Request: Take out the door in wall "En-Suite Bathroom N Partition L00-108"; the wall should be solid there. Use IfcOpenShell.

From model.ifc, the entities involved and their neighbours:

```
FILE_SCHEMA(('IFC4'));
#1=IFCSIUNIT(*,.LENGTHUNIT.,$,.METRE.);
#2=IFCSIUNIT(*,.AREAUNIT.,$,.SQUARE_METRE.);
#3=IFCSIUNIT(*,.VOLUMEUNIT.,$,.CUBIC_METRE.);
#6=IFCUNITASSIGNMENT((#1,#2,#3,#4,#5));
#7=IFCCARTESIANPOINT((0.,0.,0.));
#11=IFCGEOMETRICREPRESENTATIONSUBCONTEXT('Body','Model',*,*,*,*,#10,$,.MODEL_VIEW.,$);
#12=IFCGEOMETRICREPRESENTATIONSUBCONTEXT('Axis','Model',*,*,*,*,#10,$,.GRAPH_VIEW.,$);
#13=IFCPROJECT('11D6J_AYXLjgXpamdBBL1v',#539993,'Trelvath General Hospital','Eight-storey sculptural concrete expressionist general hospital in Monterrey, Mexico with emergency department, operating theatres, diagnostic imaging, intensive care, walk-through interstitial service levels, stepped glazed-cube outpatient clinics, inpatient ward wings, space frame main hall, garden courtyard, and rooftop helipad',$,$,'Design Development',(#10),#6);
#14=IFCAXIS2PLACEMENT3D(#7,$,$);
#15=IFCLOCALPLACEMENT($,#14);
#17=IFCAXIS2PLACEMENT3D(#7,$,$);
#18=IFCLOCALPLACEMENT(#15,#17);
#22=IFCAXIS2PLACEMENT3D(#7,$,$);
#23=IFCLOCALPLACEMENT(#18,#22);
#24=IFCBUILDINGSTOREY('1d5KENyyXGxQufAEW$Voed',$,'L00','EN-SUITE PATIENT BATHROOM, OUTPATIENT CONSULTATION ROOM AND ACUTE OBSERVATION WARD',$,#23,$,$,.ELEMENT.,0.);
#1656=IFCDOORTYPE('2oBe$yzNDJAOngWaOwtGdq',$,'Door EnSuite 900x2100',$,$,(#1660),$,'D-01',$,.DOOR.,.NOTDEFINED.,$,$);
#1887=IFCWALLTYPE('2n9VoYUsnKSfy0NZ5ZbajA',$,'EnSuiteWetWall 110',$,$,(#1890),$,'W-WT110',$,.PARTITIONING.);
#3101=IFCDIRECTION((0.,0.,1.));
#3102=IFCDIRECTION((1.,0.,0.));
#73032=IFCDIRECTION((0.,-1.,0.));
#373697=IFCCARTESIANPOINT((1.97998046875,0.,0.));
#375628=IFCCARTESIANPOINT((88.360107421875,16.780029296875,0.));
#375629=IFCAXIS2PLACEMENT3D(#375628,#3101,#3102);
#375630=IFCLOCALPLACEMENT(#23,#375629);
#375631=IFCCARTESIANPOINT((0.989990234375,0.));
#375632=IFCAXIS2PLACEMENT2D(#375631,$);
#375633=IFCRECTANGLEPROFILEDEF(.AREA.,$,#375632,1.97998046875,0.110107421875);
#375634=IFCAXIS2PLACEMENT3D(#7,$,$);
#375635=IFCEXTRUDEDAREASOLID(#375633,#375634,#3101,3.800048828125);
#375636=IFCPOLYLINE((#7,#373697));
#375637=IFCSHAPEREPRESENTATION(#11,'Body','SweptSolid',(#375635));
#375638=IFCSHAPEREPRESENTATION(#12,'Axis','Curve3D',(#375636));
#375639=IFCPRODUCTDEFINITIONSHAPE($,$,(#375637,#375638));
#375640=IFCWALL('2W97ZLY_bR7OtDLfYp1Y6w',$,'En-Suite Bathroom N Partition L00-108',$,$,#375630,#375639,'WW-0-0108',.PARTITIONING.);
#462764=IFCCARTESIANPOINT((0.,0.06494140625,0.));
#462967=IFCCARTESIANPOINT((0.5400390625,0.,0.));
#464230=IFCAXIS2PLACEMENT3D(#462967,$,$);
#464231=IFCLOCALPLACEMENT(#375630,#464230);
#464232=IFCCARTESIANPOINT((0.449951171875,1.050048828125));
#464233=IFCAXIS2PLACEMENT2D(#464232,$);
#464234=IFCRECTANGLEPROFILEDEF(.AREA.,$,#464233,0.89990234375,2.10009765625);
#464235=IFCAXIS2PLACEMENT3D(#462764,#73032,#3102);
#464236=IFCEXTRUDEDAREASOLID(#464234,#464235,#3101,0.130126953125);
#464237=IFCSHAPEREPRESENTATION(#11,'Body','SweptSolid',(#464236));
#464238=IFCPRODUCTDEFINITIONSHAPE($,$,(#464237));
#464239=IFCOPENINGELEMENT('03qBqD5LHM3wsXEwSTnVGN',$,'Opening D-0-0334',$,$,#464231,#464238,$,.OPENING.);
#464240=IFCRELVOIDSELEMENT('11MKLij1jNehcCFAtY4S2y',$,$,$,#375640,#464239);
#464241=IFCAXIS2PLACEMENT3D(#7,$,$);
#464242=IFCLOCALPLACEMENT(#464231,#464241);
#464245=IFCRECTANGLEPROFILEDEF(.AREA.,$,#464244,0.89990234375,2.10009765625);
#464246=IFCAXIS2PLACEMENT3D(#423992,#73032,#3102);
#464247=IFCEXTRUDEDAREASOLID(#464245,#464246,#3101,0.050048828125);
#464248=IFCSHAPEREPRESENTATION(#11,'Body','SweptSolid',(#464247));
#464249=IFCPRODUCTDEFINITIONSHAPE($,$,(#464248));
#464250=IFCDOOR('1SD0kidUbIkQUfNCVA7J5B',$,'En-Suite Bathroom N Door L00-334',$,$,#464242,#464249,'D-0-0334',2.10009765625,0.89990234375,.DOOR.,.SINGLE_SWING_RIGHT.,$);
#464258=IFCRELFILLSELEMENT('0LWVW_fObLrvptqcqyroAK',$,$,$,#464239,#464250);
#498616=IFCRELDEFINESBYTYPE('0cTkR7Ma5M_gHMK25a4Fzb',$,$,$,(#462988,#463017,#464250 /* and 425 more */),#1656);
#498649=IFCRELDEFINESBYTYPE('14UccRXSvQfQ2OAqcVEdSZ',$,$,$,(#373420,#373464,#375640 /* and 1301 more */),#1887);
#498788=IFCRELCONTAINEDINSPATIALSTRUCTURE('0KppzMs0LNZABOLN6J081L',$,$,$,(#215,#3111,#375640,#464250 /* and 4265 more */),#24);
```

```python
import ifcopenshell
import ifcopenshell.api.feature
import ifcopenshell.api.root
import ifcopenshell.geom
import ifcopenshell.util.shape

model = ifcopenshell.open("model.ifc")
settings = ifcopenshell.geom.settings()


def volume(element):
    """Net volume in cubic metres, openings subtracted."""
    shape = ifcopenshell.geom.create_shape(settings, element)
    return ifcopenshell.util.shape.get_volume(shape.geometry)


door = model.by_id(464250)
opening = door.FillsVoids[0].RelatingOpeningElement
wall = opening.VoidsElements[0].RelatingBuildingElement
before = volume(wall)

ifcopenshell.api.root.remove_product(model, product=door)
ifcopenshell.api.feature.remove_feature(model, feature=opening)

after = volume(wall)

print(f"wall volume {before:.3f} -> {after:.3f} m3")

model.write("model_rev.ifc")
```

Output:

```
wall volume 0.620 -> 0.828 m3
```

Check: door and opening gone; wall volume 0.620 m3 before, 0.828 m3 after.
